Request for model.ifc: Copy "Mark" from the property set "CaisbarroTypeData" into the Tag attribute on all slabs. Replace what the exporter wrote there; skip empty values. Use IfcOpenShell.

First a look at what the model holds.

```python
import ifcopenshell
import ifcopenshell.util.element

model = ifcopenshell.open("model.ifc")
print(model.schema)
slabs = model.by_type("IfcSlab")
print(len(slabs), "slabs")
for e in slabs[:8]:
    source = ifcopenshell.util.element.get_pset(e, "CaisbarroTypeData", "Mark")
    target = e.Tag
    print(e.id(), repr(source), repr(target), sep=" | ")
```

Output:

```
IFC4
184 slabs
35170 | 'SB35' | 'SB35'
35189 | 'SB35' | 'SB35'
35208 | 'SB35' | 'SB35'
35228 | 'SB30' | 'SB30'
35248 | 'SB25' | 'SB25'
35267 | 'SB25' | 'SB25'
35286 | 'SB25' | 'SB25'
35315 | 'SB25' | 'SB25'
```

```python
import ifcopenshell
import ifcopenshell.util.element

model = ifcopenshell.open("model.ifc")

count = 0
for e in model.by_type("IfcSlab"):
    value = ifcopenshell.util.element.get_pset(e, "CaisbarroTypeData", "Mark")
    current = e.Tag
    if not value or not value.strip() or current == value:
        continue
    e.Tag = value
    count += 1

print(count, "slabs updated")

model.write("model-out.ifc")
```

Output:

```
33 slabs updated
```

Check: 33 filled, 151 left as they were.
